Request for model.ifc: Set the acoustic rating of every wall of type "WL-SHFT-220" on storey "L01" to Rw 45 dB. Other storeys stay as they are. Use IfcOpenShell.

First a look at what the model holds.

```python
import ifcopenshell
import ifcopenshell.util.element

model = ifcopenshell.open("model.ifc")
print(model.schema)
storey = next(s for s in model.by_type("IfcBuildingStorey") if s.Name == "L01")
walls = [e for e in ifcopenshell.util.element.get_decomposition(storey) if e.is_a("IfcWall")]
seen = {}
for e in walls:
    element_type = ifcopenshell.util.element.get_type(e)
    key = (element_type.Name if element_type != e and element_type else None, ifcopenshell.util.element.get_pset(e, "Pset_WallCommon", "AcousticRating"))
    seen[key] = seen.get(key, 0) + 1
for (name, value), count in sorted(seen.items(), key=str):
    print(count, "x", name, "|", value)
```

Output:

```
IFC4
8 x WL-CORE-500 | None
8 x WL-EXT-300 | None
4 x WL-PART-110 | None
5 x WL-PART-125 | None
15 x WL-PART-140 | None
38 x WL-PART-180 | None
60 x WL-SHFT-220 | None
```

```python
import ifcopenshell
import ifcopenshell.api.pset
import ifcopenshell.util.element

model = ifcopenshell.open("model.ifc")

storey = next(s for s in model.by_type("IfcBuildingStorey") if s.Name == "L01")
walls = [e for e in ifcopenshell.util.element.get_decomposition(storey) if e.is_a("IfcWall")]

count = 0
for e in walls:
    element_type = ifcopenshell.util.element.get_type(e)
    if element_type in (None, e) or element_type.Name != "WL-SHFT-220":
        continue
    found = ifcopenshell.util.element.get_pset(e, "Pset_WallCommon", should_inherit=False)
    if found:
        pset = model.by_id(found["id"])
        if len(ifcopenshell.util.element.get_elements_by_pset(pset)) > 1:
            pset = ifcopenshell.api.pset.unshare_pset(model, products=[e], pset=pset)[0]
    else:
        pset = ifcopenshell.api.pset.add_pset(model, product=e, name="Pset_WallCommon")
    ifcopenshell.api.pset.edit_pset(model, pset=pset, properties={"AcousticRating": "Rw 45 dB"})
    count += 1

print(count, "walls updated")

model.write("model_rev.ifc")
```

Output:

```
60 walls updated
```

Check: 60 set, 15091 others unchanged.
